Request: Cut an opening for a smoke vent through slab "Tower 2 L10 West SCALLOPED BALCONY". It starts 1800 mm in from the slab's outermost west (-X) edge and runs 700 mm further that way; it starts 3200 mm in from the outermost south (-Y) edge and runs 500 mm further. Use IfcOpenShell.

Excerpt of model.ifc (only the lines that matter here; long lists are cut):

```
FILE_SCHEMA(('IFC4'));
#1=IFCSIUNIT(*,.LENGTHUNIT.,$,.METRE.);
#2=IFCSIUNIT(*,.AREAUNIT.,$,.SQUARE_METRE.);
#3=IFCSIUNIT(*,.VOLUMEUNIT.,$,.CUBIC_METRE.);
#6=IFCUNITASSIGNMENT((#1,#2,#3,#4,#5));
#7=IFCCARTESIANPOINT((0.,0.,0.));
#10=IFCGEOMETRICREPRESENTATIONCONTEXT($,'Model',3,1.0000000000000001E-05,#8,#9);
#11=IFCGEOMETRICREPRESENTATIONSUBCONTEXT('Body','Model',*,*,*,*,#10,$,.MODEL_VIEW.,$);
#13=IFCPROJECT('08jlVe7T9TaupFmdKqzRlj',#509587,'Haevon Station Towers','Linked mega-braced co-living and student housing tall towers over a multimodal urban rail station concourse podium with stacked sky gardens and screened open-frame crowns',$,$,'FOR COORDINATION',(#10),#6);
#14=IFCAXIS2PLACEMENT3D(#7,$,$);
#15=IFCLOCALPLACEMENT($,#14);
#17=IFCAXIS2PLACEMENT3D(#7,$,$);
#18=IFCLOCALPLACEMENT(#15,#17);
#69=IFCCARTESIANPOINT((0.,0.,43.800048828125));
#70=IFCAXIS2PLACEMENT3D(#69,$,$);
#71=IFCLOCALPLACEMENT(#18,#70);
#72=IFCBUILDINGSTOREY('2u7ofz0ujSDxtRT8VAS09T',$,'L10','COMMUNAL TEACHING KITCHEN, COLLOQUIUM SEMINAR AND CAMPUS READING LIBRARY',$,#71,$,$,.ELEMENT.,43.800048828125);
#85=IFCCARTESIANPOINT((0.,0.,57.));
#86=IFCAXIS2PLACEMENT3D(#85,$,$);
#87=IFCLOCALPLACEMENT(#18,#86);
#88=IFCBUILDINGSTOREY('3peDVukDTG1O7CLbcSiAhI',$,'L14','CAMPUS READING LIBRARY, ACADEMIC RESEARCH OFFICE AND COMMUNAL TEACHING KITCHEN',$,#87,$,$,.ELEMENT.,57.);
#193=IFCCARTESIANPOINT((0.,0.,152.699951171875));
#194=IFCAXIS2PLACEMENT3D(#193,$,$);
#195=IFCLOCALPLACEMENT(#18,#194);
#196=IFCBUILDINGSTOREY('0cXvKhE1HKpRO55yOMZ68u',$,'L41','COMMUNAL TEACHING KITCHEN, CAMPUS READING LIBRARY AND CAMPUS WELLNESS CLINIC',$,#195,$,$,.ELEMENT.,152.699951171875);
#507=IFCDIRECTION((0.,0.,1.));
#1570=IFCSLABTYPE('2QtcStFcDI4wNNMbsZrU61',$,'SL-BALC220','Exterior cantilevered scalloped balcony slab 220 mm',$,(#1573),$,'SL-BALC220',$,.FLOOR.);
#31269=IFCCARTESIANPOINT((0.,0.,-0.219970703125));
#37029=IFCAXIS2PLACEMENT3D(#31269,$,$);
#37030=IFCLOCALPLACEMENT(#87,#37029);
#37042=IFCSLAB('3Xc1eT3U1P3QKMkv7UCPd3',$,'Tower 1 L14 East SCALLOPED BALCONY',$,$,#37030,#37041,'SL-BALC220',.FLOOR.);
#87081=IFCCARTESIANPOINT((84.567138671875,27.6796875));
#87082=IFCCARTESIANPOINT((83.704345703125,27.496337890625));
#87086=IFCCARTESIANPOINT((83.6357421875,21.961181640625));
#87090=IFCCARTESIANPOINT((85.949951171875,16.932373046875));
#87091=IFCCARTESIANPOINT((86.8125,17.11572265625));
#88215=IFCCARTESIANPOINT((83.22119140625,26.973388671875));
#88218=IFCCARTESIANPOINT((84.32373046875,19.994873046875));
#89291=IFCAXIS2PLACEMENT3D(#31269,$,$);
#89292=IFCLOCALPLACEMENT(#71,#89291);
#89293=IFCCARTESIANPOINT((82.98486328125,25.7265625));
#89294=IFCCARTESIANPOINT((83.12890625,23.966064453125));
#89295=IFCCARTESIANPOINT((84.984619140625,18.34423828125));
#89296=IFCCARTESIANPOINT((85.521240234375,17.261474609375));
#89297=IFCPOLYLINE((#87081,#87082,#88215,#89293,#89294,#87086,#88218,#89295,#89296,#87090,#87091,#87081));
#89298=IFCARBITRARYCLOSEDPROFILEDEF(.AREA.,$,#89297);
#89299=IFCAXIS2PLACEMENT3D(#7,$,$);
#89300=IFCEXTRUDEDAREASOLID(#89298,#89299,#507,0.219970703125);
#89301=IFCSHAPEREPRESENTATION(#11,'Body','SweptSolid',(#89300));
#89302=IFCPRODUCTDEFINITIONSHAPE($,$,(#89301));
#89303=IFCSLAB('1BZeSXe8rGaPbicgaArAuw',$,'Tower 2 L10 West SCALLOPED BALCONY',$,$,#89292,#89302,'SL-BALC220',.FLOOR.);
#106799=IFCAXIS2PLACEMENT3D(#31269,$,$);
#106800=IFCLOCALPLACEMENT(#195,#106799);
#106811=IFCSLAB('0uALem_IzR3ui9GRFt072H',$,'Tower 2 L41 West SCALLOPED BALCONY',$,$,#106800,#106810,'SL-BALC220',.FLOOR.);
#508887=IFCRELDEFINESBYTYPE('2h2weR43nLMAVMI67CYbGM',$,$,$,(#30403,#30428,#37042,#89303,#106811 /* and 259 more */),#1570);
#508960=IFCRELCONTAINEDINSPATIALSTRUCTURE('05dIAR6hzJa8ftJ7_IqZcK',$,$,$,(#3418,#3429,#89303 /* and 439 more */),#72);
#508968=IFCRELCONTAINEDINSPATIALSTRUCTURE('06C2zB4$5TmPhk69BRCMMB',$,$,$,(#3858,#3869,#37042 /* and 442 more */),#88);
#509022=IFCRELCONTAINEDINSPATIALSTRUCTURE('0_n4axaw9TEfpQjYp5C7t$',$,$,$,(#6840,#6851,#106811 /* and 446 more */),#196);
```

```python
import numpy as np
import ifcopenshell
import ifcopenshell.api.feature
import ifcopenshell.api.geometry
import ifcopenshell.api.root
import ifcopenshell.geom
import ifcopenshell.util.placement
import ifcopenshell.util.representation
import ifcopenshell.util.shape
import ifcopenshell.util.unit

model = ifcopenshell.open("model.ifc")
unit_scale = ifcopenshell.util.unit.calculate_unit_scale(model)
settings = ifcopenshell.geom.settings()


def volume(element):
    """Net volume in cubic metres, openings subtracted."""
    shape = ifcopenshell.geom.create_shape(settings, element)
    return ifcopenshell.util.shape.get_volume(shape.geometry)


slab = model.by_guid("1BZeSXe8rGaPbicgaArAuw")
before = volume(slab)

# Extent in the slab's own axes, in metres. The edges named are its -X and -Y sides.
slab_shape = ifcopenshell.geom.create_shape(settings, slab)
vertices = ifcopenshell.util.shape.get_vertices(slab_shape.geometry)
x_min, y_min, bottom = vertices.min(axis=0)
top = vertices[:, 2].max()

opening = ifcopenshell.api.root.create_entity(model, ifc_class="IfcOpeningElement", name="Smoke vent opening", predefined_type="OPENING")
context = ifcopenshell.util.representation.get_context(model, "Model", "Body", "MODEL_VIEW")
width, depth = 0.7, 0.5
outline = [(0.0, 0.0), (width, 0.0), (width, depth), (0.0, depth), (0.0, 0.0)]
# Overshoot both faces by 50 mm so the cut is clean.
shape = ifcopenshell.api.geometry.add_slab_representation(
    model, context=context, depth=top - bottom + 0.1, polyline=outline
)
ifcopenshell.api.geometry.assign_representation(model, product=opening, representation=shape)

matrix = ifcopenshell.util.placement.get_local_placement(slab.ObjectPlacement)
matrix[:, 3] = matrix @ np.append(np.array([x_min + 1.8, y_min + 3.2, bottom - 0.05]) / unit_scale, 1.0)
ifcopenshell.api.geometry.edit_object_placement(model, product=opening, matrix=matrix, is_si=False)
ifcopenshell.api.feature.add_feature(model, feature=opening, element=slab)

after = volume(slab)

print(f"slab volume {before:.3f} -> {after:.3f} m3")

model.write("model_v2.ifc")
```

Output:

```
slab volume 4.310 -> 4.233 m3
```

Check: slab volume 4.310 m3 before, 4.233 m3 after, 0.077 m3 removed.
